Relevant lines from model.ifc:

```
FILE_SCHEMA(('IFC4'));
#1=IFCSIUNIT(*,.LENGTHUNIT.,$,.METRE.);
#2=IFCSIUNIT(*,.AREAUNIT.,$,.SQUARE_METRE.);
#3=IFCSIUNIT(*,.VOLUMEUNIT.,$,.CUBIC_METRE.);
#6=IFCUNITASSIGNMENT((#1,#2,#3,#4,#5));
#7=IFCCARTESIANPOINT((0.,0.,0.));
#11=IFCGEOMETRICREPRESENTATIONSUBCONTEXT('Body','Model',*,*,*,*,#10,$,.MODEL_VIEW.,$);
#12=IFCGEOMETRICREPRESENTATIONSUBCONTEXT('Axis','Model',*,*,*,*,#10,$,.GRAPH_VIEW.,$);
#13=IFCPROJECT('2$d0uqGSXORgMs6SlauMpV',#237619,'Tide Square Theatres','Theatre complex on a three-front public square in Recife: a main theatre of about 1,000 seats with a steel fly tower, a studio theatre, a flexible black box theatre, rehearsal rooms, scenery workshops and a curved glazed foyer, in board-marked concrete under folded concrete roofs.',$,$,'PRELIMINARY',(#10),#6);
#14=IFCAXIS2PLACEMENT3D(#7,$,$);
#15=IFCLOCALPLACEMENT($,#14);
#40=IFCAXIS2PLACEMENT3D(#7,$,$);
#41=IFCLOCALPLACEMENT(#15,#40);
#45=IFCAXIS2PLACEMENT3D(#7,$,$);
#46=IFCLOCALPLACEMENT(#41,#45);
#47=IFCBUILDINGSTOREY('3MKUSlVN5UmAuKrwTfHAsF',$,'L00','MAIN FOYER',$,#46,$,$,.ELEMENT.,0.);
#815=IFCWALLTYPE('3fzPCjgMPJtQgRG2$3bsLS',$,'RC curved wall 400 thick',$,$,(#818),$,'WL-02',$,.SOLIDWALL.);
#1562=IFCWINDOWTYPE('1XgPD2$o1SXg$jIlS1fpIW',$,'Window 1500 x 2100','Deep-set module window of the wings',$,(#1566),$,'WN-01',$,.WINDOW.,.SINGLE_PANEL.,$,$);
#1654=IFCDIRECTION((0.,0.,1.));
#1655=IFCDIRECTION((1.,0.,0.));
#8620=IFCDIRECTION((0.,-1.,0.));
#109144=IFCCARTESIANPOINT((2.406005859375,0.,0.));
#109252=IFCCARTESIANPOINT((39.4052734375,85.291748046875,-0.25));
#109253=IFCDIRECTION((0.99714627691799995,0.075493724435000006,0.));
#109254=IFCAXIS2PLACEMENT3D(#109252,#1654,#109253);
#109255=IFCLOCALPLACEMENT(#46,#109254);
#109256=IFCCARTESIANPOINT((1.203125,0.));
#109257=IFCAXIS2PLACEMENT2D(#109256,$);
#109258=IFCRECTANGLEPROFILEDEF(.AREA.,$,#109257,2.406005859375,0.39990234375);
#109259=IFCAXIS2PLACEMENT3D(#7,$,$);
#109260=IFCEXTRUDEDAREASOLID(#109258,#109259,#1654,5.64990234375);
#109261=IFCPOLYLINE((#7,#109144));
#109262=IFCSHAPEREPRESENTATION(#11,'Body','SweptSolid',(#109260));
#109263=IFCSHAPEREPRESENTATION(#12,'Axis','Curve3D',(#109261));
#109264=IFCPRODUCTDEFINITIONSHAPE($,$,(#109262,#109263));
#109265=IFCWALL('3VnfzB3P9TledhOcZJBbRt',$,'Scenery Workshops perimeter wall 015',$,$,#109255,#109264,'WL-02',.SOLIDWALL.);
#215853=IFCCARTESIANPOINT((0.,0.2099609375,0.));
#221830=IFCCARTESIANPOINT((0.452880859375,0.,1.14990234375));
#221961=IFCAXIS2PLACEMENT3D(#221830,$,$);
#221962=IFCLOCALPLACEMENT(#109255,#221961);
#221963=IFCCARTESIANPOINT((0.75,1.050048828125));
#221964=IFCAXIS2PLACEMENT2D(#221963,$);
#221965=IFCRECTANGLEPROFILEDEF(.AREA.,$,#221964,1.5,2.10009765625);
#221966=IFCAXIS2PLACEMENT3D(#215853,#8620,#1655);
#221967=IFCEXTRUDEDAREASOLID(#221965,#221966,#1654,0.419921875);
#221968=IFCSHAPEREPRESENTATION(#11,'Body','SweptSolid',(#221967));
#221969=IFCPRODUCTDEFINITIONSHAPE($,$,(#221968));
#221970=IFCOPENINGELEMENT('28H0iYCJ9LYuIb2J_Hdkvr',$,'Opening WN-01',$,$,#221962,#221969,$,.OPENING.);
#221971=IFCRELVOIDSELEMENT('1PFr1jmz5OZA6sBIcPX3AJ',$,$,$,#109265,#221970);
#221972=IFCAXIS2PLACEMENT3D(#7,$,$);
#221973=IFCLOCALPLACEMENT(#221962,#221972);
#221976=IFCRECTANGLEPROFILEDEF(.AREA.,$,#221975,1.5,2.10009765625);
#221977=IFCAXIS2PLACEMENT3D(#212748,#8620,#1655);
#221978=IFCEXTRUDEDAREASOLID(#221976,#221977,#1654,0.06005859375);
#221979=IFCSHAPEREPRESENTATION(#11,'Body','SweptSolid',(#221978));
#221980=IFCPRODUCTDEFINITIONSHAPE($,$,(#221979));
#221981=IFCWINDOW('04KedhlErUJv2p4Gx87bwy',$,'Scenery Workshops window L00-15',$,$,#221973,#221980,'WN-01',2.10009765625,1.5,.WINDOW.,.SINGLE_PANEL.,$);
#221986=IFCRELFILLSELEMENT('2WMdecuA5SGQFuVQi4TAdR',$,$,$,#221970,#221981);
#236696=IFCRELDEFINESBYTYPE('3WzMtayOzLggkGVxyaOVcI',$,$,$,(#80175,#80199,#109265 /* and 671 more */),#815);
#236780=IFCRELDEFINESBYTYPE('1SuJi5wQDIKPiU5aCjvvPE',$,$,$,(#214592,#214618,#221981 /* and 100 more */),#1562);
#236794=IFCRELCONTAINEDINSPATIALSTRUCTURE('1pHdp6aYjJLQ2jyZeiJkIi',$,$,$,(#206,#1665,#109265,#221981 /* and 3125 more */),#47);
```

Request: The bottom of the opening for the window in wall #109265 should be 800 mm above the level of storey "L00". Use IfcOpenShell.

```python
import numpy as np
import ifcopenshell
import ifcopenshell.api.geometry
import ifcopenshell.geom
import ifcopenshell.util.element
import ifcopenshell.util.placement
import ifcopenshell.util.shape
import ifcopenshell.util.unit

model = ifcopenshell.open("model.ifc")
unit_scale = ifcopenshell.util.unit.calculate_unit_scale(model)

window = model.by_guid("04KedhlErUJv2p4Gx87bwy")
opening = window.FillsVoids[0].RelatingOpeningElement
storey = ifcopenshell.util.element.get_container(window, ifc_class="IfcBuildingStorey")
level = ifcopenshell.util.placement.get_local_placement(storey.ObjectPlacement)[2, 3]

# The opening's origin need not be at the sill, so measure its lowest point.
shape = ifcopenshell.geom.create_shape(ifcopenshell.geom.settings(), opening)
bottom = ifcopenshell.util.shape.get_shape_bottom_elevation(shape, shape.geometry) / unit_scale
dz = level + 0.8 - bottom

shift = np.array([0.0, 0.0, dz])
# The window is placed relative to its opening, so it follows when the opening moves.
matrix = ifcopenshell.util.placement.get_local_placement(opening.ObjectPlacement)
matrix[:3, 3] += shift
ifcopenshell.api.geometry.edit_object_placement(
    model, product=opening, matrix=matrix, is_si=False, should_transform_children=True
)

print(f"moved by {dz * unit_scale:+.3f} m")

model.write("model-out.ifc")
```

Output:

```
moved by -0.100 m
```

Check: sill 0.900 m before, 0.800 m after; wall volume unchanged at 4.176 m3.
